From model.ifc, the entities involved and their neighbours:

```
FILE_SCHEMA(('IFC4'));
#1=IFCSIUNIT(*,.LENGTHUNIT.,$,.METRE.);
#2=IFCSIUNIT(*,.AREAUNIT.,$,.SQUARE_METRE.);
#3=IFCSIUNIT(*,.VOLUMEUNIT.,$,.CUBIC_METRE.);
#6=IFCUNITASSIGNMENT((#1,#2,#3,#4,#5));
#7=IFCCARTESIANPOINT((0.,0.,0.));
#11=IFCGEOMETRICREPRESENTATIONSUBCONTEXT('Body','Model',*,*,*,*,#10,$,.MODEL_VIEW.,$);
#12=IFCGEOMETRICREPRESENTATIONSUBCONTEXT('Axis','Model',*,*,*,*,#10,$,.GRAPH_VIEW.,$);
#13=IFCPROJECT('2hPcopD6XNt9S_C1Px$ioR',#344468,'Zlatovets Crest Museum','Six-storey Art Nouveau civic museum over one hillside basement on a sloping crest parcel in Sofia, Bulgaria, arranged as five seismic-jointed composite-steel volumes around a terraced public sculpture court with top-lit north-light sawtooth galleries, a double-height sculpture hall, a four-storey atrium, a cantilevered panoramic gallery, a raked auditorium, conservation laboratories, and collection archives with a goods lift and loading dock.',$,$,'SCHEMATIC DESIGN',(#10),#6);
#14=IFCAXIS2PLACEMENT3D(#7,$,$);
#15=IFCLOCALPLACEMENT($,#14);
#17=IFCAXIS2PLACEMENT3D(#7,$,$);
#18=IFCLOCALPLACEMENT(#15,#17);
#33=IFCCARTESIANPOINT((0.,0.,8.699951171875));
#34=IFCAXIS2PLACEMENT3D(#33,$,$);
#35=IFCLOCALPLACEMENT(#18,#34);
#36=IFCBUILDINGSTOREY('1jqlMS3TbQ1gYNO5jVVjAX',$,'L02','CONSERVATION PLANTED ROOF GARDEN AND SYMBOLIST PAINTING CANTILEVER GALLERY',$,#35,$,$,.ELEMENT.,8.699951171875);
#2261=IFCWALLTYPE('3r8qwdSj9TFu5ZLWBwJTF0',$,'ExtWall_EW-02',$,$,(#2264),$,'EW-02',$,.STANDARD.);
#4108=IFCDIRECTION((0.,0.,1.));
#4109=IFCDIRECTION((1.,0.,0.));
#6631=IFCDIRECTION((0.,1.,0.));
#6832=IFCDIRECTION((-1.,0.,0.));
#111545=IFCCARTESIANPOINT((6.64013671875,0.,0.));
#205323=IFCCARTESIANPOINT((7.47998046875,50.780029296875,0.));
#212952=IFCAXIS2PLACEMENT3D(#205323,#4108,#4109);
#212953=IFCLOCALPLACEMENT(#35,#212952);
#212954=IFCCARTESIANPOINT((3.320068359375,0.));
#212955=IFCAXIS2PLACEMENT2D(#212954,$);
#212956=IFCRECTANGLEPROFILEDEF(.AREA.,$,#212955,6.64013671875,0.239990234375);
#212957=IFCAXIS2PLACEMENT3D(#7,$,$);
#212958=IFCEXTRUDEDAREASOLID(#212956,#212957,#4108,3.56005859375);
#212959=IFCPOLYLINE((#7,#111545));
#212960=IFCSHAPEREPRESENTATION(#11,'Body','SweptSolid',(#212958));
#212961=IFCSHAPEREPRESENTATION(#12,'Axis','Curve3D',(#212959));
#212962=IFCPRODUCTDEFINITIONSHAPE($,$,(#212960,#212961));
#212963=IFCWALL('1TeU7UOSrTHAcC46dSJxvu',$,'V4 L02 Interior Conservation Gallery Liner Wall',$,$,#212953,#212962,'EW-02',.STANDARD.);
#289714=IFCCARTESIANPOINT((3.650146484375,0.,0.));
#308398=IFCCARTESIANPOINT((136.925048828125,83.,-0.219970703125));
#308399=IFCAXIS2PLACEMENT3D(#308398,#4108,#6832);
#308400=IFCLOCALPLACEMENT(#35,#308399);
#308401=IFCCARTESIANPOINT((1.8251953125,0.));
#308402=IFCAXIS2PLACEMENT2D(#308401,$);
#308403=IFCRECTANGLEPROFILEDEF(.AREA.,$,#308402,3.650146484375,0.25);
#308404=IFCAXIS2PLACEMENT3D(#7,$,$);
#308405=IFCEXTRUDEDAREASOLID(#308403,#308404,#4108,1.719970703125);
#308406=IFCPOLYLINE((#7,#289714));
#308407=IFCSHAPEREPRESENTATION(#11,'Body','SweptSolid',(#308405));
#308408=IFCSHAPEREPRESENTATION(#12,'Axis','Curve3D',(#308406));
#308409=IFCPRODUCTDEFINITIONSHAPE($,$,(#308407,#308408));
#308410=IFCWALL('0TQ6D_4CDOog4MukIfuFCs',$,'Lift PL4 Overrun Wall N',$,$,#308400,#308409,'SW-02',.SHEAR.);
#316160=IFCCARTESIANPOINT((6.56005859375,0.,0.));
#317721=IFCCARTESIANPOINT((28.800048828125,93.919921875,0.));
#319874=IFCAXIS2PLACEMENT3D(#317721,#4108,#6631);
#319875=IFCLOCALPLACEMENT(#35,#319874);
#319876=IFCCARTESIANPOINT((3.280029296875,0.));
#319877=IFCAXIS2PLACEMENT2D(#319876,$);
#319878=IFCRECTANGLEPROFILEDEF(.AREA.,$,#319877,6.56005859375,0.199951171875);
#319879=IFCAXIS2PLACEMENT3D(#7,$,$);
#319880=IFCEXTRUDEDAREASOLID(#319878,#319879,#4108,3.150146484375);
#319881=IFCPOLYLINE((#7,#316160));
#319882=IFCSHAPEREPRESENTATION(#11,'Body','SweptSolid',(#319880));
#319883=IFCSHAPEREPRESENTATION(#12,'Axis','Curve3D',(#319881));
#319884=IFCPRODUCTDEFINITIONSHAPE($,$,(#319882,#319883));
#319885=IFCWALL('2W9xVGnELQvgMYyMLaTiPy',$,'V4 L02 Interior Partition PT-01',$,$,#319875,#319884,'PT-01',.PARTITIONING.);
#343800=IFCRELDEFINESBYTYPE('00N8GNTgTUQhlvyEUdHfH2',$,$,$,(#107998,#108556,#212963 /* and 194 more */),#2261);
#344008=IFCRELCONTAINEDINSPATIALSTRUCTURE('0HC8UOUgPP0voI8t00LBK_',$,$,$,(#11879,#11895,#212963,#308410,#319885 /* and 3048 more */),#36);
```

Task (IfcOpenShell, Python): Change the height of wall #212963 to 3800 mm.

```python
import ifcopenshell
import ifcopenshell.geom
import ifcopenshell.util.representation
import ifcopenshell.util.shape

model = ifcopenshell.open("model.ifc")
settings = ifcopenshell.geom.settings()


def volume(element):
    """Net volume in cubic metres, openings subtracted."""
    shape = ifcopenshell.geom.create_shape(settings, element)
    return ifcopenshell.util.shape.get_volume(shape.geometry)


wall = model.by_guid("1TeU7UOSrTHAcC46dSJxvu")
before = volume(wall)

body = ifcopenshell.util.representation.get_representation(wall, "Model", "Body")
solid = body.Items[0]
old_height = solid.Depth
solid.Depth = 3.8
after = volume(wall)

print(f"height {old_height:g} -> {solid.Depth:g}, volume {before:.3f} -> {after:.3f} m3")

model.write("model_edited.ifc")
```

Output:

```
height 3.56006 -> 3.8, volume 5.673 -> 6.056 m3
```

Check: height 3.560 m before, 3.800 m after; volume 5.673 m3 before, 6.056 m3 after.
